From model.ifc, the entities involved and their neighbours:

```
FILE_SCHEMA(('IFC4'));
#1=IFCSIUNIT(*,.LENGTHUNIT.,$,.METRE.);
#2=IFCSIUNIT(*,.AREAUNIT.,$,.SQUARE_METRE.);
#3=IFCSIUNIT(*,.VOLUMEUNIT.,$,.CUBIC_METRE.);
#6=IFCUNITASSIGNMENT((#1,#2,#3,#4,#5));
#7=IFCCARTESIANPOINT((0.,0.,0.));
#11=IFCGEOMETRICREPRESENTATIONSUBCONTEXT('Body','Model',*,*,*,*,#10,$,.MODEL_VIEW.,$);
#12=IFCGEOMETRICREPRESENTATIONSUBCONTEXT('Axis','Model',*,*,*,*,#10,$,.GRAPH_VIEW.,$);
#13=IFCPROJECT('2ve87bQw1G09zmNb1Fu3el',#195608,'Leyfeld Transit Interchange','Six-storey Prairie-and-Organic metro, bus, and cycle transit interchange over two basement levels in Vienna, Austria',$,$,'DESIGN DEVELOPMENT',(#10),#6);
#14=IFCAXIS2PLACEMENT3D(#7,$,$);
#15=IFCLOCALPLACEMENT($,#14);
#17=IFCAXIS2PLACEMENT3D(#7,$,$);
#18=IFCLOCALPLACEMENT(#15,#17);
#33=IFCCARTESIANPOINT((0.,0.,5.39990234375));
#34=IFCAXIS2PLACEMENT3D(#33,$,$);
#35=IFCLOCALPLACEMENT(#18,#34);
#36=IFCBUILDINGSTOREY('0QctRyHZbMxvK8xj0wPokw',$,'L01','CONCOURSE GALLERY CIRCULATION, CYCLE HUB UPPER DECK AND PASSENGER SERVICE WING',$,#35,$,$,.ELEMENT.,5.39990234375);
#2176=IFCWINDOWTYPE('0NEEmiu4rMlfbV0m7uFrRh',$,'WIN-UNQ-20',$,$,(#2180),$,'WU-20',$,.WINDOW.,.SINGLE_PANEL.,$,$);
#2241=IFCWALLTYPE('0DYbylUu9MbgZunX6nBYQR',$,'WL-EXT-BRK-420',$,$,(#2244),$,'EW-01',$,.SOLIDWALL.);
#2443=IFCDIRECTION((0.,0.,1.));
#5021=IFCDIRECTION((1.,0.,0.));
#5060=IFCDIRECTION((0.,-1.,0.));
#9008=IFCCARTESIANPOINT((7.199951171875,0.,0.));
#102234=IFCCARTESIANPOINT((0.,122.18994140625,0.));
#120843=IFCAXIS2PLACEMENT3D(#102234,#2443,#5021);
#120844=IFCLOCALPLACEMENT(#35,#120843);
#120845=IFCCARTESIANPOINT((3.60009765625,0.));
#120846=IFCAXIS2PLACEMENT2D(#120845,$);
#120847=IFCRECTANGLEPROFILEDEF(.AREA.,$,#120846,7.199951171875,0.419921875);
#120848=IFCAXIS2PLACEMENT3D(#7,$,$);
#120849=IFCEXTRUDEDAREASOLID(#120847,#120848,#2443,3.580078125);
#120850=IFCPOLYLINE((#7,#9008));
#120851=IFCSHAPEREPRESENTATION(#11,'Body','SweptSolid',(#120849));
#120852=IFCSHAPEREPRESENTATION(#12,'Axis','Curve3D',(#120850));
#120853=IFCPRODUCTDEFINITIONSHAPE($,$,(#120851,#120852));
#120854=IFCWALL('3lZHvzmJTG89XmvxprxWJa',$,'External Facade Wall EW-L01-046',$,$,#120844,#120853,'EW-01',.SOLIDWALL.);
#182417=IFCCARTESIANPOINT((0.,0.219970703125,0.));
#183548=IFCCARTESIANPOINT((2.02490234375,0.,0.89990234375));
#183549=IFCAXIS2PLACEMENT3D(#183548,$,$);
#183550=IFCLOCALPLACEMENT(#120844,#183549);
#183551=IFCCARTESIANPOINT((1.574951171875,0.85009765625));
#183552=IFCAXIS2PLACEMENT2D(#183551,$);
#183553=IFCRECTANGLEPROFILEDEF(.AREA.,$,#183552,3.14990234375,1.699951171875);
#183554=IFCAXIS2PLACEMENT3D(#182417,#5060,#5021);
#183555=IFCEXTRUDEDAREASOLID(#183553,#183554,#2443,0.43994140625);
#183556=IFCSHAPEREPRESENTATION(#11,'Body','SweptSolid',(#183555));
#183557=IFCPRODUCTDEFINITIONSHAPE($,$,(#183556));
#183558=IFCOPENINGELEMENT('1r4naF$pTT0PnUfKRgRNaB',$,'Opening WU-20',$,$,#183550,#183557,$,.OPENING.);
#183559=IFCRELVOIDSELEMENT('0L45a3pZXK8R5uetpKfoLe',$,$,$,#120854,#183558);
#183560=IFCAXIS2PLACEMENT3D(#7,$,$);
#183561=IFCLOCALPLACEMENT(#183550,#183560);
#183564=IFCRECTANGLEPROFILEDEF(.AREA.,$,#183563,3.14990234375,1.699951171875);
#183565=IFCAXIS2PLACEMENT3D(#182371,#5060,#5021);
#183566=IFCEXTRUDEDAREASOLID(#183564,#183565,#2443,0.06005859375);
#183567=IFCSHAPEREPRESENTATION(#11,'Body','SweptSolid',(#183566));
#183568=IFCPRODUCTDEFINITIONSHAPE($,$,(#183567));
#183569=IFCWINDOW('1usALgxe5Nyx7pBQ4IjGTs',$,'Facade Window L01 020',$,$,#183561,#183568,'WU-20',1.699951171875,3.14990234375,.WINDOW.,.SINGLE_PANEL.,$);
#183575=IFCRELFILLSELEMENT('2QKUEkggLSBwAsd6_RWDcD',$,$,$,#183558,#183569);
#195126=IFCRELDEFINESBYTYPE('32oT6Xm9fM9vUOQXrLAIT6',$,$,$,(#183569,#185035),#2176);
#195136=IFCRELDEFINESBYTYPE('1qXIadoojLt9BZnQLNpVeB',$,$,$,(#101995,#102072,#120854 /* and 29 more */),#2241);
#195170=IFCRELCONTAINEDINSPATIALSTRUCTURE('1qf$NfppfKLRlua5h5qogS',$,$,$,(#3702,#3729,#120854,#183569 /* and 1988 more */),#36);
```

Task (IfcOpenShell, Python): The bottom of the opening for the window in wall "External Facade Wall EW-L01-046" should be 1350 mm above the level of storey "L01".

```python
import numpy as np
import ifcopenshell
import ifcopenshell.api.geometry
import ifcopenshell.geom
import ifcopenshell.util.element
import ifcopenshell.util.placement
import ifcopenshell.util.shape
import ifcopenshell.util.unit

model = ifcopenshell.open("model.ifc")
unit_scale = ifcopenshell.util.unit.calculate_unit_scale(model)

window = model.by_guid("1usALgxe5Nyx7pBQ4IjGTs")
opening = window.FillsVoids[0].RelatingOpeningElement
storey = ifcopenshell.util.element.get_container(window, ifc_class="IfcBuildingStorey")
level = ifcopenshell.util.placement.get_local_placement(storey.ObjectPlacement)[2, 3]

# The opening's origin need not be at the sill, so measure its lowest point.
shape = ifcopenshell.geom.create_shape(ifcopenshell.geom.settings(), opening)
bottom = ifcopenshell.util.shape.get_shape_bottom_elevation(shape, shape.geometry) / unit_scale
dz = level + 1.35 - bottom

shift = np.array([0.0, 0.0, dz])
# The window is placed relative to its opening, so it follows when the opening moves.
matrix = ifcopenshell.util.placement.get_local_placement(opening.ObjectPlacement)
matrix[:3, 3] += shift
ifcopenshell.api.geometry.edit_object_placement(
    model, product=opening, matrix=matrix, is_si=False, should_transform_children=True
)

print(f"moved by {dz * unit_scale:+.3f} m")

model.write("model_edited.ifc")
```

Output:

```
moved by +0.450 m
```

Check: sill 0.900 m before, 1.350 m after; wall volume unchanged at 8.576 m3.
